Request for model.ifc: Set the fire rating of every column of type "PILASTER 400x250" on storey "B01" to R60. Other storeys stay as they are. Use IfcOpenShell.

First a look at what the model holds.

```python
import ifcopenshell
import ifcopenshell.util.element

model = ifcopenshell.open("model.ifc")
print(model.schema)
storey = next(s for s in model.by_type("IfcBuildingStorey") if s.Name == "B01")
columns = [e for e in ifcopenshell.util.element.get_decomposition(storey) if e.is_a("IfcColumn")]
seen = {}
for e in columns:
    element_type = ifcopenshell.util.element.get_type(e)
    key = (element_type.Name if element_type != e and element_type else None, ifcopenshell.util.element.get_pset(e, "Pset_ColumnCommon", "FireRating"))
    seen[key] = seen.get(key, 0) + 1
for (name, value), count in sorted(seen.items(), key=str):
    print(count, "x", name, "|", value)
```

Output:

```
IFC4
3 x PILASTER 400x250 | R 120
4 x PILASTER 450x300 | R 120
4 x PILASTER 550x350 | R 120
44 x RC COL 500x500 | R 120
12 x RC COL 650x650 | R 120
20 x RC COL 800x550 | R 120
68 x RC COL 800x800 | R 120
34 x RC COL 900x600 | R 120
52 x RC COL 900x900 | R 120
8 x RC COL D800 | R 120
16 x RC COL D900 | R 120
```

```python
import ifcopenshell
import ifcopenshell.api.pset
import ifcopenshell.util.element

model = ifcopenshell.open("model.ifc")

storey = next(s for s in model.by_type("IfcBuildingStorey") if s.Name == "B01")
columns = [e for e in ifcopenshell.util.element.get_decomposition(storey) if e.is_a("IfcColumn")]

count = 0
for e in columns:
    element_type = ifcopenshell.util.element.get_type(e)
    if element_type in (None, e) or element_type.Name != "PILASTER 400x250":
        continue
    # add_pset returns the element's existing set when there is one.
    pset = ifcopenshell.api.pset.add_pset(model, product=e, name="Pset_ColumnCommon")
    ifcopenshell.api.pset.edit_pset(model, pset=pset, properties={"FireRating": "R60"})
    count += 1

print(count, "columns updated")

model.write("model_v2.ifc")
```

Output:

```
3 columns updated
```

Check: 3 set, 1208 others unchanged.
